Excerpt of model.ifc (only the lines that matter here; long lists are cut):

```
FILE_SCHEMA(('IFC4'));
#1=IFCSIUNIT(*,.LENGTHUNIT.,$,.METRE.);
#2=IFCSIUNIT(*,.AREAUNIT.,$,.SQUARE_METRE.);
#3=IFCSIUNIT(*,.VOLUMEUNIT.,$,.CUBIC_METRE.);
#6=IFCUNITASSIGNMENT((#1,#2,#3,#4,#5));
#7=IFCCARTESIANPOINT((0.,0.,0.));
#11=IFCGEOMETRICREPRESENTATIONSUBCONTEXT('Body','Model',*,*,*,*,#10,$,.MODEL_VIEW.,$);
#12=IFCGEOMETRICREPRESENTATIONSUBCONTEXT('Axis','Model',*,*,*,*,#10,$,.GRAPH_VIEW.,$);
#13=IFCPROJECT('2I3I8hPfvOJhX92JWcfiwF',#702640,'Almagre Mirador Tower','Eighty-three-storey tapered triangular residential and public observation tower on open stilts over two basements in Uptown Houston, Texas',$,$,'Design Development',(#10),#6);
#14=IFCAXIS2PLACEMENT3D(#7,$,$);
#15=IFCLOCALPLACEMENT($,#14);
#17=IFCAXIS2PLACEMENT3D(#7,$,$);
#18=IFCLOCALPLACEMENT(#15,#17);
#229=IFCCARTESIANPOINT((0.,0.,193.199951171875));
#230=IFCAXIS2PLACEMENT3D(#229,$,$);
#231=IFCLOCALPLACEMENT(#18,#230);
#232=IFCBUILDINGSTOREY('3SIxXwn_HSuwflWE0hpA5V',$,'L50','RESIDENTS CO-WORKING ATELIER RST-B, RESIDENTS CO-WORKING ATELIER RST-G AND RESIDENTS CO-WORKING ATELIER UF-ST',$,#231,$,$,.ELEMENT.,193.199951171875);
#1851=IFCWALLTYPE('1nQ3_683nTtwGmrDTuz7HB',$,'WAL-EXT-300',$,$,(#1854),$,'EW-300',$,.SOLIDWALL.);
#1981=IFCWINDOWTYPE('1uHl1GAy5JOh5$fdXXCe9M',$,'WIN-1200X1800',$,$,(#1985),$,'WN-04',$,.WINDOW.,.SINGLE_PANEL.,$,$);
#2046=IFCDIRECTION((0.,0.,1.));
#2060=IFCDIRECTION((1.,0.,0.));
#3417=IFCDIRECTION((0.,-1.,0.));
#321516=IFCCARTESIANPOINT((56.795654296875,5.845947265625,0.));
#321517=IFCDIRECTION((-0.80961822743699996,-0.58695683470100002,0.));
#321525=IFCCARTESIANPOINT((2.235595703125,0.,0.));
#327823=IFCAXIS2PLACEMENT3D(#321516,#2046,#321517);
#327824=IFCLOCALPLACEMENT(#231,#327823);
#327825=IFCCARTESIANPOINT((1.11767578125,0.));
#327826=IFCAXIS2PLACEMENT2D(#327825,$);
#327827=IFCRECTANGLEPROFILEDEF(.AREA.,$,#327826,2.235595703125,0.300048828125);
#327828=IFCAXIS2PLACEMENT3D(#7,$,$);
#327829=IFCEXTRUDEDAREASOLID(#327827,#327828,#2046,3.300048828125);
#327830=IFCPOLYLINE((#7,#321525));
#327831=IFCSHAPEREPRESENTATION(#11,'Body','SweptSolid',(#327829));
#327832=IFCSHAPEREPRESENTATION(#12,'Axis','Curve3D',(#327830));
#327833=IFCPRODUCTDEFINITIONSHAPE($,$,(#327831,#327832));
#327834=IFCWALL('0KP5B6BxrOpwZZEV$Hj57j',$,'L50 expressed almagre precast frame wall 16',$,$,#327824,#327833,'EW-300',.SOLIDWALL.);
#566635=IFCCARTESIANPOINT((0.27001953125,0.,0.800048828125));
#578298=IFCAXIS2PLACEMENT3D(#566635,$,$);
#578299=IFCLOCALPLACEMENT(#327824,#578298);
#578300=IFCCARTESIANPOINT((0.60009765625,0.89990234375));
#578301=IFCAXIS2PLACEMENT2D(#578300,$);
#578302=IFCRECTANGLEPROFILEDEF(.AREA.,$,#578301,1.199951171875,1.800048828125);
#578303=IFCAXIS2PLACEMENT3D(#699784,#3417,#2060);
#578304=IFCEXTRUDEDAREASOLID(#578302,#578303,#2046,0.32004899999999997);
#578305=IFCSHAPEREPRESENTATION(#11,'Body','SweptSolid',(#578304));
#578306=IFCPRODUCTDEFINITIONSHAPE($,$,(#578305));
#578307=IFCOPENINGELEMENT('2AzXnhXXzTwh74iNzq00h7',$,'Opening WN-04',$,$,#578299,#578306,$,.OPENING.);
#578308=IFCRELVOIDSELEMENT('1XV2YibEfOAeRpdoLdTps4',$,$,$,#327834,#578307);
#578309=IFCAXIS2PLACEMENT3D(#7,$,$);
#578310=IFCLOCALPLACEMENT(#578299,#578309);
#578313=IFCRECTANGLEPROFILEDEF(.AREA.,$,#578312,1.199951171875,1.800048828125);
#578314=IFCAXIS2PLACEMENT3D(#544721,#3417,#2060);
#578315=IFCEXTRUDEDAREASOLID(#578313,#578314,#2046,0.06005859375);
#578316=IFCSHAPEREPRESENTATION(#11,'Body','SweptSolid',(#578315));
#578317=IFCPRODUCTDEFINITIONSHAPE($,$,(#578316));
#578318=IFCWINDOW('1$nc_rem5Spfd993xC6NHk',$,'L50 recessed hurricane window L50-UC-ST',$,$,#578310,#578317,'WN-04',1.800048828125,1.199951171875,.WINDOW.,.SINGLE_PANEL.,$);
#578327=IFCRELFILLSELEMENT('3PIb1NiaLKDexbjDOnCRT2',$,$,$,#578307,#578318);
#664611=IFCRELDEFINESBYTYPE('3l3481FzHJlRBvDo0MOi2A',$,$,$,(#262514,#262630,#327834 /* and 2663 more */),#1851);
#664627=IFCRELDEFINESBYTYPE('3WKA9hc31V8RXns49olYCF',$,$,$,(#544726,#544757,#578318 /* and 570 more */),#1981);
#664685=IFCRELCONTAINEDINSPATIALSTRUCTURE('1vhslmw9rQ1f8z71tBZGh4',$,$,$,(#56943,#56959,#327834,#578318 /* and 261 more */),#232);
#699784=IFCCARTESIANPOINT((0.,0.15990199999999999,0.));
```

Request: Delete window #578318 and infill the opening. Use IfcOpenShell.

```python
import ifcopenshell
import ifcopenshell.api.feature
import ifcopenshell.api.root
import ifcopenshell.geom
import ifcopenshell.util.shape

model = ifcopenshell.open("model.ifc")
settings = ifcopenshell.geom.settings()


def volume(element):
    """Net volume in cubic metres, openings subtracted."""
    shape = ifcopenshell.geom.create_shape(settings, element)
    return ifcopenshell.util.shape.get_volume(shape.geometry)


window = model.by_guid("1$nc_rem5Spfd993xC6NHk")
opening = window.FillsVoids[0].RelatingOpeningElement
wall = opening.VoidsElements[0].RelatingBuildingElement
before = volume(wall)

ifcopenshell.api.root.remove_product(model, product=window)
ifcopenshell.api.feature.remove_feature(model, feature=opening)

after = volume(wall)

print(f"wall volume {before:.3f} -> {after:.3f} m3")

model.write("model_rev.ifc")
```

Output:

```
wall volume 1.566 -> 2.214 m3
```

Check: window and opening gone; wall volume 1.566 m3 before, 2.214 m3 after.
